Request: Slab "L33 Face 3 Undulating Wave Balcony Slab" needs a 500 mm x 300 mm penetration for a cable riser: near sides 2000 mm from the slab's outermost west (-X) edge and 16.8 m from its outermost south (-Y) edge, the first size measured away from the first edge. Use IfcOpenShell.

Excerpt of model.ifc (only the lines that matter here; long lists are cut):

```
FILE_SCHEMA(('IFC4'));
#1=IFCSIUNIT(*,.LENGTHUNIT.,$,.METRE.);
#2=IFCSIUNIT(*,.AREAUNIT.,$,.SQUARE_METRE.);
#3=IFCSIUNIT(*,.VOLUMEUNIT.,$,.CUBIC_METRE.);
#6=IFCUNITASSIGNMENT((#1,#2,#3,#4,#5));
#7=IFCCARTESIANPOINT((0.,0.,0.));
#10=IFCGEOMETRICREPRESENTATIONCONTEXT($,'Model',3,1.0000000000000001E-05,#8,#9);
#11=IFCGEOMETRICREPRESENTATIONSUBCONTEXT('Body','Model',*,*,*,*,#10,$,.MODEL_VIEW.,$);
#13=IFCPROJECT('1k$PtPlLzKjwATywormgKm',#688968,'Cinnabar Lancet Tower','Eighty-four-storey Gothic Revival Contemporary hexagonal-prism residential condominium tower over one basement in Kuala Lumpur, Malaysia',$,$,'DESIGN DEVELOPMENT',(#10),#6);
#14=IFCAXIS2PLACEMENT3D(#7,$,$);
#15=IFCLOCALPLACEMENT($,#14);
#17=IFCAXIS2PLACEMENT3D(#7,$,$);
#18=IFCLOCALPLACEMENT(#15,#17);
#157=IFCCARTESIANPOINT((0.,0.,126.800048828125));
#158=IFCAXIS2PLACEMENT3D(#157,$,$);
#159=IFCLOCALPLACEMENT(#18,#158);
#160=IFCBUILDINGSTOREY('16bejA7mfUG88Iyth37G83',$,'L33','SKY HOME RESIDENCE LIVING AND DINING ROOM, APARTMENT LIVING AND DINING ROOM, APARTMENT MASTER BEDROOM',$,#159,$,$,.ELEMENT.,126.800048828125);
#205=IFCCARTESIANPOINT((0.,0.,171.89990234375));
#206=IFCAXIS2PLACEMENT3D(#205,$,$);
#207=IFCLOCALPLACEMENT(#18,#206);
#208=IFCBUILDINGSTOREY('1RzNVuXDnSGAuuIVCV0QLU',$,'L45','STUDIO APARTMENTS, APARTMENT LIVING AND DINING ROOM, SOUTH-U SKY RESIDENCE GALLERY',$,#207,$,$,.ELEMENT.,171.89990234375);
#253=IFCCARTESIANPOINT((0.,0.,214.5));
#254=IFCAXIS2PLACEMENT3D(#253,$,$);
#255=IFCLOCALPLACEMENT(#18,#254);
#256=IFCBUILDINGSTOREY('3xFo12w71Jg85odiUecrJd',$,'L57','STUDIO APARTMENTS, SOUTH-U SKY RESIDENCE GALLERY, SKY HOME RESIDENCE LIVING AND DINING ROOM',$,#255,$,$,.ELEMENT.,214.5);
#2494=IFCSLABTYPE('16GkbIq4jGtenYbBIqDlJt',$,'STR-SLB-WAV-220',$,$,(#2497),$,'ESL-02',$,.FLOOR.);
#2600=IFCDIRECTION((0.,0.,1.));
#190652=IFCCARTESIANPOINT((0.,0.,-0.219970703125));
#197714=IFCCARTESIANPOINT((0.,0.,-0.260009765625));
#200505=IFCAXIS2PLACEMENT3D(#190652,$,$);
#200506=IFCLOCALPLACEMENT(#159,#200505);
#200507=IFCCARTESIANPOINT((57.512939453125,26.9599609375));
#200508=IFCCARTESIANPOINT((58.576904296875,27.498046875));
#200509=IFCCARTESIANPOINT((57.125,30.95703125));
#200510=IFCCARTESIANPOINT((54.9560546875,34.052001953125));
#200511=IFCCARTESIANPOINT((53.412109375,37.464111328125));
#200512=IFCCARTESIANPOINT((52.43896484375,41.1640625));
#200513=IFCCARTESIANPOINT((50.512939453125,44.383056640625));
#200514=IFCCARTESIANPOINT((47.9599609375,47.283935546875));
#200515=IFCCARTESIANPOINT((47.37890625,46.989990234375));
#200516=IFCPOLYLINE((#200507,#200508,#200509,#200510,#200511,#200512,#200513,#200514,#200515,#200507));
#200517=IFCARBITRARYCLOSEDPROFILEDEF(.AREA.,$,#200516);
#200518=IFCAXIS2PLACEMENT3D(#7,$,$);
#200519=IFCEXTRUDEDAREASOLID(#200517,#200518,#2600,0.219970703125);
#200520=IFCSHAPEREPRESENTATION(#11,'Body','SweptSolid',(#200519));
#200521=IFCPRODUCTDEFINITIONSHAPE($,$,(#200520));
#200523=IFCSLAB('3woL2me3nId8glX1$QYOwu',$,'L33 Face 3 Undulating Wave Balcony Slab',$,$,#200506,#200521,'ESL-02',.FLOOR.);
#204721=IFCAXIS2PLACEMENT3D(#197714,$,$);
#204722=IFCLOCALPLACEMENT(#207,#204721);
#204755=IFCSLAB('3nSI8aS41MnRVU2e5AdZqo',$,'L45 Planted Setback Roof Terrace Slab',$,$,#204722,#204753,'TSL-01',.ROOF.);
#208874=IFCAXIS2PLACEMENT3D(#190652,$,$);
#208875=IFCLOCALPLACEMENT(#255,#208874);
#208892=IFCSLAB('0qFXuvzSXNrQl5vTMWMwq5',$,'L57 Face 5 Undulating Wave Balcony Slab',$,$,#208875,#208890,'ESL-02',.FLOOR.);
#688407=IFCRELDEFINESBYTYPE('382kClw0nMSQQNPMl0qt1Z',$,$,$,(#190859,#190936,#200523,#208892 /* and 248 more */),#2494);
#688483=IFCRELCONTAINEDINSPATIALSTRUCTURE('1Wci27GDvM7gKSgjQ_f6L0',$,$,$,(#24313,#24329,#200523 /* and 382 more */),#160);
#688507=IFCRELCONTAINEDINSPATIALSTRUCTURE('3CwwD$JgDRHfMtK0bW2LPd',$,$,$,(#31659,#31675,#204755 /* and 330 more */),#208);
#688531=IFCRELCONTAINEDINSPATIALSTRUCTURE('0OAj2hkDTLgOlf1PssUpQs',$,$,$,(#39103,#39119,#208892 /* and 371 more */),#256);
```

```python
import numpy as np
import ifcopenshell
import ifcopenshell.api.feature
import ifcopenshell.api.geometry
import ifcopenshell.api.root
import ifcopenshell.geom
import ifcopenshell.util.placement
import ifcopenshell.util.representation
import ifcopenshell.util.shape
import ifcopenshell.util.unit

model = ifcopenshell.open("model.ifc")
unit_scale = ifcopenshell.util.unit.calculate_unit_scale(model)
settings = ifcopenshell.geom.settings()


def volume(element):
    """Net volume in cubic metres, openings subtracted."""
    shape = ifcopenshell.geom.create_shape(settings, element)
    return ifcopenshell.util.shape.get_volume(shape.geometry)


slab = model.by_guid("3woL2me3nId8glX1$QYOwu")
before = volume(slab)

# Extent in the slab's own axes, in metres. The edges named are its -X and -Y sides.
slab_shape = ifcopenshell.geom.create_shape(settings, slab)
vertices = ifcopenshell.util.shape.get_vertices(slab_shape.geometry)
x_min, y_min, bottom = vertices.min(axis=0)
top = vertices[:, 2].max()

opening = ifcopenshell.api.root.create_entity(model, ifc_class="IfcOpeningElement", name="Cable riser opening", predefined_type="OPENING")
context = ifcopenshell.util.representation.get_context(model, "Model", "Body", "MODEL_VIEW")
width, depth = 0.5, 0.3
outline = [(0.0, 0.0), (width, 0.0), (width, depth), (0.0, depth), (0.0, 0.0)]
# Overshoot both faces by 50 mm so the cut is clean.
shape = ifcopenshell.api.geometry.add_slab_representation(
    model, context=context, depth=top - bottom + 0.1, polyline=outline
)
ifcopenshell.api.geometry.assign_representation(model, product=opening, representation=shape)

matrix = ifcopenshell.util.placement.get_local_placement(slab.ObjectPlacement)
matrix[:, 3] = matrix @ np.append(np.array([x_min + 2, y_min + 16.8, bottom - 0.05]) / unit_scale, 1.0)
ifcopenshell.api.geometry.edit_object_placement(model, product=opening, matrix=matrix, is_si=False)
ifcopenshell.api.feature.add_feature(model, feature=opening, element=slab)

after = volume(slab)

print(f"slab volume {before:.3f} -> {after:.3f} m3")

model.write("model_v2.ifc")
```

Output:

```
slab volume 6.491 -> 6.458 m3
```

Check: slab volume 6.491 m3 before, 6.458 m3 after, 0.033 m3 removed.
